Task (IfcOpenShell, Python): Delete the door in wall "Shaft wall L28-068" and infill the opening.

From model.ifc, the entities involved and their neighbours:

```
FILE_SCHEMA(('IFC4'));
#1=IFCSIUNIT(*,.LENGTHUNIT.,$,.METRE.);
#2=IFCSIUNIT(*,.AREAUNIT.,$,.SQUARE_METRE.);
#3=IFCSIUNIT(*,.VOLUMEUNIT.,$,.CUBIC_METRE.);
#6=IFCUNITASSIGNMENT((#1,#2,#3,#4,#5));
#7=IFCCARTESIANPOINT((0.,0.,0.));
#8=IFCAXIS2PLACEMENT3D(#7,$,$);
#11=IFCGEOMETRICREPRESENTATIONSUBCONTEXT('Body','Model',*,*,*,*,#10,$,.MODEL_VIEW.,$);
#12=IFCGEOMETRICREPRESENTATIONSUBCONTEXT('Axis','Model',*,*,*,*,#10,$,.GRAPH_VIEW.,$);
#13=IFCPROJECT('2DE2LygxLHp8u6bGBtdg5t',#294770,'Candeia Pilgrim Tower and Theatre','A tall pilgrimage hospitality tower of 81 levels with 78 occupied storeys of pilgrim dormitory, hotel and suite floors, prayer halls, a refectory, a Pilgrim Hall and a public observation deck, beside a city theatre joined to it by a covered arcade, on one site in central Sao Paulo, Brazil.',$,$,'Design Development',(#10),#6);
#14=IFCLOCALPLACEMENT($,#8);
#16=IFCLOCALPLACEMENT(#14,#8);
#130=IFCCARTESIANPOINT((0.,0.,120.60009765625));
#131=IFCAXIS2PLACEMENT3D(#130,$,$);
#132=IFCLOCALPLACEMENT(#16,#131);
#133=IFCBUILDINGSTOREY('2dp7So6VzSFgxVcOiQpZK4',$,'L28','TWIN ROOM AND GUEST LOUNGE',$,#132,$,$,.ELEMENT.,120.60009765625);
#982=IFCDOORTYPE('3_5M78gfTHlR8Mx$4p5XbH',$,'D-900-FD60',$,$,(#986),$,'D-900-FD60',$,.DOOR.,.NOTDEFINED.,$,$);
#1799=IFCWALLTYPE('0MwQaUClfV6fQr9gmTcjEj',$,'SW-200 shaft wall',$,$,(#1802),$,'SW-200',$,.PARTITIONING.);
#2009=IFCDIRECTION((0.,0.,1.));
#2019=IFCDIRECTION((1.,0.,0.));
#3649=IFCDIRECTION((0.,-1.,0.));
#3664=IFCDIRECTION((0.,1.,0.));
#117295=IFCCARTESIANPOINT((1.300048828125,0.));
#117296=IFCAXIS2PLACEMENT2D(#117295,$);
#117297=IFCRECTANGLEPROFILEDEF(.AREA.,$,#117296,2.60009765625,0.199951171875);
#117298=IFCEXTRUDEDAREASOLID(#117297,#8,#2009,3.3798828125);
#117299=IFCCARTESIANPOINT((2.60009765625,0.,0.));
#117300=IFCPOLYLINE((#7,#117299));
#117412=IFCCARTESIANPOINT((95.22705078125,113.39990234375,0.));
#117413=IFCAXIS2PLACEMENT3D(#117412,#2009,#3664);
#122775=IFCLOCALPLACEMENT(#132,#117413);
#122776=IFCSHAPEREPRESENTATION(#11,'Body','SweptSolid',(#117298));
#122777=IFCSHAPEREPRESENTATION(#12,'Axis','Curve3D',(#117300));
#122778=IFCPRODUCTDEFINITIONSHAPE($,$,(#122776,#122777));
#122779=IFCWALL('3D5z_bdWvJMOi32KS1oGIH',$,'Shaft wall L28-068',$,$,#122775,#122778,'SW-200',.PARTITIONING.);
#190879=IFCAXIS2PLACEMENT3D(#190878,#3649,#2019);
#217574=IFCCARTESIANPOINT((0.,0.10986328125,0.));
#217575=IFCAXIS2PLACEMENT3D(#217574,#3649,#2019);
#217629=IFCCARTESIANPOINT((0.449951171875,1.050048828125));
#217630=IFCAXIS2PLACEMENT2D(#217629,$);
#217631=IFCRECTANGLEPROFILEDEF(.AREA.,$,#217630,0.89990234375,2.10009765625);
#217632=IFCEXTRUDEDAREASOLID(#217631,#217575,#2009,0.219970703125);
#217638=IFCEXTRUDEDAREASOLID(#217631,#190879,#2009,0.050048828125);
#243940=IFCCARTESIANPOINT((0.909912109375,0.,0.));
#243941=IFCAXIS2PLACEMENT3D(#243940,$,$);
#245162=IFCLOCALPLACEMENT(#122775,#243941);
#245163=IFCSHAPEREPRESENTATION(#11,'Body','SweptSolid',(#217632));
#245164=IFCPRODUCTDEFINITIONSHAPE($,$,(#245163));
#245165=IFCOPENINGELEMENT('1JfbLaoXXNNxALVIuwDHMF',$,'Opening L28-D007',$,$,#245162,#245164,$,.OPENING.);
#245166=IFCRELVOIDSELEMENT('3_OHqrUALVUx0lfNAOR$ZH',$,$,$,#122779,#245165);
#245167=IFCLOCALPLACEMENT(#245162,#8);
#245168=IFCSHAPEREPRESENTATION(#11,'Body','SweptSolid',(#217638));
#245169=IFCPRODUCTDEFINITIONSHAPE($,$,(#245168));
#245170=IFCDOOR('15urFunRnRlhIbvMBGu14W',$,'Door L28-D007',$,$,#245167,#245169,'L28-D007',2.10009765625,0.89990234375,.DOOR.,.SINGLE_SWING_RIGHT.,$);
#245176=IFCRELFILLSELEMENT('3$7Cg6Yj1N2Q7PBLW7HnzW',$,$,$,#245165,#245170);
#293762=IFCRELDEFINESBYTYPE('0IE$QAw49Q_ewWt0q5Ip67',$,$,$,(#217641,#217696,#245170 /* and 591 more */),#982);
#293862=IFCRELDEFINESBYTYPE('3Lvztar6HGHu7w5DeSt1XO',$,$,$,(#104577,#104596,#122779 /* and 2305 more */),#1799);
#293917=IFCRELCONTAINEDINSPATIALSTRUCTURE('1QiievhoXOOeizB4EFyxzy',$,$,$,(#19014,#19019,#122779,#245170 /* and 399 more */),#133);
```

```python
import ifcopenshell
import ifcopenshell.api.feature
import ifcopenshell.api.root
import ifcopenshell.geom
import ifcopenshell.util.shape

model = ifcopenshell.open("model.ifc")
settings = ifcopenshell.geom.settings()


def volume(element):
    """Net volume in cubic metres, openings subtracted."""
    shape = ifcopenshell.geom.create_shape(settings, element)
    return ifcopenshell.util.shape.get_volume(shape.geometry)


door = model.by_id(245170)
opening = door.FillsVoids[0].RelatingOpeningElement
wall = opening.VoidsElements[0].RelatingBuildingElement
before = volume(wall)

ifcopenshell.api.root.remove_product(model, product=door)
ifcopenshell.api.feature.remove_feature(model, feature=opening)

after = volume(wall)

print(f"wall volume {before:.3f} -> {after:.3f} m3")

model.write("model_updated.ifc")
```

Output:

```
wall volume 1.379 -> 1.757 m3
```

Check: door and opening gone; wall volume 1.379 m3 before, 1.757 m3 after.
